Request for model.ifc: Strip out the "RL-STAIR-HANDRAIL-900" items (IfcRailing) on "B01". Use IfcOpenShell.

First a look at what the model holds.

```python
import ifcopenshell
import ifcopenshell.util.element

model = ifcopenshell.open("model.ifc")
print(model.schema)
storey = next(s for s in model.by_type("IfcBuildingStorey") if s.Name == "B01")
railings = [e for e in ifcopenshell.util.element.get_decomposition(storey) if e.is_a("IfcRailing")]
seen = {}
for e in railings:
    element_type = ifcopenshell.util.element.get_type(e)
    name = element_type.Name if element_type not in (None, e) else None
    seen[name] = seen.get(name, 0) + 1
for name, count in sorted(seen.items(), key=str):
    print(count, "x", name)
```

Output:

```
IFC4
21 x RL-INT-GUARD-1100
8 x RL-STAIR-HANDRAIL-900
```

```python
import ifcopenshell
import ifcopenshell.api.root
import ifcopenshell.util.element

model = ifcopenshell.open("model.ifc")

storey = next(s for s in model.by_type("IfcBuildingStorey") if s.Name == "B01")
railings = [e for e in ifcopenshell.util.element.get_decomposition(storey) if e.is_a("IfcRailing")]
targets = [e for e in railings if (t := ifcopenshell.util.element.get_type(e)) not in (None, e) and t.Name == "RL-STAIR-HANDRAIL-900"]

for e in targets:
    ifcopenshell.api.root.remove_product(model, product=e)
print(len(targets), "removed")

model.write("model_edited.ifc")
```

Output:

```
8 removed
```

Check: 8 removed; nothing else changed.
